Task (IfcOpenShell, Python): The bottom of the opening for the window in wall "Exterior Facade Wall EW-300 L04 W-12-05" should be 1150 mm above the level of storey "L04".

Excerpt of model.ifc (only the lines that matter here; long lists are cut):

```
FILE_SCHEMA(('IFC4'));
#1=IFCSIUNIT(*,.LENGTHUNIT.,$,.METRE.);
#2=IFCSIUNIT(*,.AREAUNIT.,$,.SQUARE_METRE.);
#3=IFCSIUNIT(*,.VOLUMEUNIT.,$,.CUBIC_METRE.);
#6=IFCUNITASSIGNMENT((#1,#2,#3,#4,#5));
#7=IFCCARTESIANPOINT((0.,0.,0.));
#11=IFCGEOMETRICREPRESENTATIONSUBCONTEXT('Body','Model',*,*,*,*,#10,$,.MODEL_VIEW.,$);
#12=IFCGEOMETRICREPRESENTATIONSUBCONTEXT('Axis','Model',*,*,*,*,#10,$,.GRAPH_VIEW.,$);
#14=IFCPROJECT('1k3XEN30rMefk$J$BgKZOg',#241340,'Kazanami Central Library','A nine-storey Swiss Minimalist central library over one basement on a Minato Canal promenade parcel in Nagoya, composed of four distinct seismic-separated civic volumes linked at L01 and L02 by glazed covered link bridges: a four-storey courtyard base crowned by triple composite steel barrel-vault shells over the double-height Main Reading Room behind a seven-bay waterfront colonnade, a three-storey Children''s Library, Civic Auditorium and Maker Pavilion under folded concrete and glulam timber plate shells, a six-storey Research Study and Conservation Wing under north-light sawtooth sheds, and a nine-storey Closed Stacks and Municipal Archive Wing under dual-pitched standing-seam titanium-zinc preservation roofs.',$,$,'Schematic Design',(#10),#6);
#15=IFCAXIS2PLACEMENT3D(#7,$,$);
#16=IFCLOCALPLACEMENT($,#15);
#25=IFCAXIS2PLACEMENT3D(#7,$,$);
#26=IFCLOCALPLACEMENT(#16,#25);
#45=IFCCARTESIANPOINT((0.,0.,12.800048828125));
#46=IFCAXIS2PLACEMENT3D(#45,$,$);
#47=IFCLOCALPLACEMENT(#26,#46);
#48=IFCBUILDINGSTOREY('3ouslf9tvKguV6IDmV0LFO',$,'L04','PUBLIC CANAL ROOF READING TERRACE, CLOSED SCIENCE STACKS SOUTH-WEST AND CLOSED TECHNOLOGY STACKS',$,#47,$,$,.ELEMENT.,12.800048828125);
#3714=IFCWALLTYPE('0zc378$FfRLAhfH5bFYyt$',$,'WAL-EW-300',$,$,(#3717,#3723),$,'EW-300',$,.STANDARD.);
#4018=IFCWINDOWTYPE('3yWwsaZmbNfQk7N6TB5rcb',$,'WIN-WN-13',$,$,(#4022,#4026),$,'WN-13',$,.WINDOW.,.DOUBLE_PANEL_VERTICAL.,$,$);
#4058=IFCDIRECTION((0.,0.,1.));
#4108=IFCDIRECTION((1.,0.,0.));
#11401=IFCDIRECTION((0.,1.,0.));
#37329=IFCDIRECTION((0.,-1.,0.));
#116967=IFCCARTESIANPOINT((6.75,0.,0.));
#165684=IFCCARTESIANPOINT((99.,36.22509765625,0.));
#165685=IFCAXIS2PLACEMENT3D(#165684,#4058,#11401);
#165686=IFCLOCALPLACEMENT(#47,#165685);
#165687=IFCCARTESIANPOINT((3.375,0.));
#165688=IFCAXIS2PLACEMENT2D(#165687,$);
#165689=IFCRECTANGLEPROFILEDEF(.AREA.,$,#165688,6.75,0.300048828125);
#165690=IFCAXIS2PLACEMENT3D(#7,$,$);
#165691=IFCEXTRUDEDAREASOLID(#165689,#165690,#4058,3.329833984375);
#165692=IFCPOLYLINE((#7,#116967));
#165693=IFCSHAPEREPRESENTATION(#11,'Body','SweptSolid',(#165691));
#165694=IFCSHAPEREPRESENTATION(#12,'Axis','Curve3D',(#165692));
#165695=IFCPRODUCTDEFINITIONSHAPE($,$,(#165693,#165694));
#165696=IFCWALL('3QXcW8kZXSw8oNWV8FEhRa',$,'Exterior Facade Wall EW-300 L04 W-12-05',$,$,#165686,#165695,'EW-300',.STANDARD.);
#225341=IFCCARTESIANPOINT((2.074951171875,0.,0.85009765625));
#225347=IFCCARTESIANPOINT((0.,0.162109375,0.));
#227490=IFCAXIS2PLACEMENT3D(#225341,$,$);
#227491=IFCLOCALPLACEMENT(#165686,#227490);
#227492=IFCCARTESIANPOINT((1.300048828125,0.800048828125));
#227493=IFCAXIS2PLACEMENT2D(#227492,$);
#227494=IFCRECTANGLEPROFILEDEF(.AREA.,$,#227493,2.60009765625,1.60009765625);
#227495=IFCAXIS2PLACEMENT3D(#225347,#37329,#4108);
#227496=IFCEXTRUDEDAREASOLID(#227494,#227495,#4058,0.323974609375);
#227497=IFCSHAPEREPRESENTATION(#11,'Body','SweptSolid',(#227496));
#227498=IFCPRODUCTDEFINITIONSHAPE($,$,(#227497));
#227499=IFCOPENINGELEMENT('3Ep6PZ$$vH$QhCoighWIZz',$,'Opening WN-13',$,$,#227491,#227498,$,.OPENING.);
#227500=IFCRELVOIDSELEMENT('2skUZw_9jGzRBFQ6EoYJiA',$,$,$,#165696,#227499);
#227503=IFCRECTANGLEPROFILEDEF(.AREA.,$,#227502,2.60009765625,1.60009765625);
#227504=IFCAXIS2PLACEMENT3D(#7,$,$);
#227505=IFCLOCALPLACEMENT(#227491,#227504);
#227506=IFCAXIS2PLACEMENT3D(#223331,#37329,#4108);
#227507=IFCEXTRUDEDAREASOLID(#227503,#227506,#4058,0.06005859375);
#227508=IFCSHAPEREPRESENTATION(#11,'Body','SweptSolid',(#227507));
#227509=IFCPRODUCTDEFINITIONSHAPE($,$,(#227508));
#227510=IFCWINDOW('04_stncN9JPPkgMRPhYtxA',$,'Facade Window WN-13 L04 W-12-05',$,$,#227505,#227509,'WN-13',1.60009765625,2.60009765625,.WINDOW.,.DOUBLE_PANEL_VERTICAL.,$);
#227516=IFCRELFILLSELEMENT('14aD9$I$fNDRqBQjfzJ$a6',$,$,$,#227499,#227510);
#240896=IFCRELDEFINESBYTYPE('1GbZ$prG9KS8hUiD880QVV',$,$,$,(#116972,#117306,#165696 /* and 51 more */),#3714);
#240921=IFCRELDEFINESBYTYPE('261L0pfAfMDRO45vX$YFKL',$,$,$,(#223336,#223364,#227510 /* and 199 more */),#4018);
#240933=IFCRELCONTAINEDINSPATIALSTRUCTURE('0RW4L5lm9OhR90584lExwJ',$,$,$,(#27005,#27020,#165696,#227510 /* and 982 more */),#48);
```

```python
import numpy as np
import ifcopenshell
import ifcopenshell.api.geometry
import ifcopenshell.geom
import ifcopenshell.util.element
import ifcopenshell.util.placement
import ifcopenshell.util.shape
import ifcopenshell.util.unit

model = ifcopenshell.open("model.ifc")
unit_scale = ifcopenshell.util.unit.calculate_unit_scale(model)

window = model.by_guid("04_stncN9JPPkgMRPhYtxA")
opening = window.FillsVoids[0].RelatingOpeningElement
storey = ifcopenshell.util.element.get_container(window, ifc_class="IfcBuildingStorey")
level = ifcopenshell.util.placement.get_local_placement(storey.ObjectPlacement)[2, 3]

# The opening's origin need not be at the sill, so measure its lowest point.
shape = ifcopenshell.geom.create_shape(ifcopenshell.geom.settings(), opening)
bottom = ifcopenshell.util.shape.get_shape_bottom_elevation(shape, shape.geometry) / unit_scale
dz = level + 1.15 - bottom

shift = np.array([0.0, 0.0, dz])
# The window is placed relative to its opening, so it follows when the opening moves.
matrix = ifcopenshell.util.placement.get_local_placement(opening.ObjectPlacement)
matrix[:3, 3] += shift
ifcopenshell.api.geometry.edit_object_placement(
    model, product=opening, matrix=matrix, is_si=False, should_transform_children=True
)

print(f"moved by {dz * unit_scale:+.3f} m")

model.write("model-out.ifc")
```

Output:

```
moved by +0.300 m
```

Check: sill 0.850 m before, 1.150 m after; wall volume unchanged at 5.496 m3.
